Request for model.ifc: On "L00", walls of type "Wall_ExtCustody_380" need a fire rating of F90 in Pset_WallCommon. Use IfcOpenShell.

First a look at what the model holds.

```python
import ifcopenshell
import ifcopenshell.util.element

model = ifcopenshell.open("model.ifc")
print(model.schema)
storey = next(s for s in model.by_type("IfcBuildingStorey") if s.Name == "L00")
walls = [e for e in ifcopenshell.util.element.get_decomposition(storey) if e.is_a("IfcWall")]
seen = {}
for e in walls:
    element_type = ifcopenshell.util.element.get_type(e)
    key = (element_type.Name if element_type != e and element_type else None, ifcopenshell.util.element.get_pset(e, "Pset_WallCommon", "FireRating"))
    seen[key] = seen.get(key, 0) + 1
for (name, value), count in sorted(seen.items(), key=str):
    print(count, "x", name, "|", value)
```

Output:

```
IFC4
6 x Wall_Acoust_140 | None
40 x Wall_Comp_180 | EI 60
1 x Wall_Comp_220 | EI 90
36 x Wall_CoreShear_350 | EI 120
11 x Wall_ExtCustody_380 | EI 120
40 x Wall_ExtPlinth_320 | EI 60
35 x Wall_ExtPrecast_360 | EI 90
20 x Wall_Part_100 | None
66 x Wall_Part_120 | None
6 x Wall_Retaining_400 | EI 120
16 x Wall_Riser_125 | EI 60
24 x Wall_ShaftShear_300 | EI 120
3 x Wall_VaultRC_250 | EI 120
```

```python
import ifcopenshell
import ifcopenshell.api.pset
import ifcopenshell.util.element

model = ifcopenshell.open("model.ifc")

storey = next(s for s in model.by_type("IfcBuildingStorey") if s.Name == "L00")
walls = [e for e in ifcopenshell.util.element.get_decomposition(storey) if e.is_a("IfcWall")]

count = 0
for e in walls:
    element_type = ifcopenshell.util.element.get_type(e)
    if element_type in (None, e) or element_type.Name != "Wall_ExtCustody_380":
        continue
    # add_pset returns the element's existing set when there is one.
    pset = ifcopenshell.api.pset.add_pset(model, product=e, name="Pset_WallCommon")
    ifcopenshell.api.pset.edit_pset(model, pset=pset, properties={"FireRating": "F90"})
    count += 1

print(count, "walls updated")

model.write("model-out.ifc")
```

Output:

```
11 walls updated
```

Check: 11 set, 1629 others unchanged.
